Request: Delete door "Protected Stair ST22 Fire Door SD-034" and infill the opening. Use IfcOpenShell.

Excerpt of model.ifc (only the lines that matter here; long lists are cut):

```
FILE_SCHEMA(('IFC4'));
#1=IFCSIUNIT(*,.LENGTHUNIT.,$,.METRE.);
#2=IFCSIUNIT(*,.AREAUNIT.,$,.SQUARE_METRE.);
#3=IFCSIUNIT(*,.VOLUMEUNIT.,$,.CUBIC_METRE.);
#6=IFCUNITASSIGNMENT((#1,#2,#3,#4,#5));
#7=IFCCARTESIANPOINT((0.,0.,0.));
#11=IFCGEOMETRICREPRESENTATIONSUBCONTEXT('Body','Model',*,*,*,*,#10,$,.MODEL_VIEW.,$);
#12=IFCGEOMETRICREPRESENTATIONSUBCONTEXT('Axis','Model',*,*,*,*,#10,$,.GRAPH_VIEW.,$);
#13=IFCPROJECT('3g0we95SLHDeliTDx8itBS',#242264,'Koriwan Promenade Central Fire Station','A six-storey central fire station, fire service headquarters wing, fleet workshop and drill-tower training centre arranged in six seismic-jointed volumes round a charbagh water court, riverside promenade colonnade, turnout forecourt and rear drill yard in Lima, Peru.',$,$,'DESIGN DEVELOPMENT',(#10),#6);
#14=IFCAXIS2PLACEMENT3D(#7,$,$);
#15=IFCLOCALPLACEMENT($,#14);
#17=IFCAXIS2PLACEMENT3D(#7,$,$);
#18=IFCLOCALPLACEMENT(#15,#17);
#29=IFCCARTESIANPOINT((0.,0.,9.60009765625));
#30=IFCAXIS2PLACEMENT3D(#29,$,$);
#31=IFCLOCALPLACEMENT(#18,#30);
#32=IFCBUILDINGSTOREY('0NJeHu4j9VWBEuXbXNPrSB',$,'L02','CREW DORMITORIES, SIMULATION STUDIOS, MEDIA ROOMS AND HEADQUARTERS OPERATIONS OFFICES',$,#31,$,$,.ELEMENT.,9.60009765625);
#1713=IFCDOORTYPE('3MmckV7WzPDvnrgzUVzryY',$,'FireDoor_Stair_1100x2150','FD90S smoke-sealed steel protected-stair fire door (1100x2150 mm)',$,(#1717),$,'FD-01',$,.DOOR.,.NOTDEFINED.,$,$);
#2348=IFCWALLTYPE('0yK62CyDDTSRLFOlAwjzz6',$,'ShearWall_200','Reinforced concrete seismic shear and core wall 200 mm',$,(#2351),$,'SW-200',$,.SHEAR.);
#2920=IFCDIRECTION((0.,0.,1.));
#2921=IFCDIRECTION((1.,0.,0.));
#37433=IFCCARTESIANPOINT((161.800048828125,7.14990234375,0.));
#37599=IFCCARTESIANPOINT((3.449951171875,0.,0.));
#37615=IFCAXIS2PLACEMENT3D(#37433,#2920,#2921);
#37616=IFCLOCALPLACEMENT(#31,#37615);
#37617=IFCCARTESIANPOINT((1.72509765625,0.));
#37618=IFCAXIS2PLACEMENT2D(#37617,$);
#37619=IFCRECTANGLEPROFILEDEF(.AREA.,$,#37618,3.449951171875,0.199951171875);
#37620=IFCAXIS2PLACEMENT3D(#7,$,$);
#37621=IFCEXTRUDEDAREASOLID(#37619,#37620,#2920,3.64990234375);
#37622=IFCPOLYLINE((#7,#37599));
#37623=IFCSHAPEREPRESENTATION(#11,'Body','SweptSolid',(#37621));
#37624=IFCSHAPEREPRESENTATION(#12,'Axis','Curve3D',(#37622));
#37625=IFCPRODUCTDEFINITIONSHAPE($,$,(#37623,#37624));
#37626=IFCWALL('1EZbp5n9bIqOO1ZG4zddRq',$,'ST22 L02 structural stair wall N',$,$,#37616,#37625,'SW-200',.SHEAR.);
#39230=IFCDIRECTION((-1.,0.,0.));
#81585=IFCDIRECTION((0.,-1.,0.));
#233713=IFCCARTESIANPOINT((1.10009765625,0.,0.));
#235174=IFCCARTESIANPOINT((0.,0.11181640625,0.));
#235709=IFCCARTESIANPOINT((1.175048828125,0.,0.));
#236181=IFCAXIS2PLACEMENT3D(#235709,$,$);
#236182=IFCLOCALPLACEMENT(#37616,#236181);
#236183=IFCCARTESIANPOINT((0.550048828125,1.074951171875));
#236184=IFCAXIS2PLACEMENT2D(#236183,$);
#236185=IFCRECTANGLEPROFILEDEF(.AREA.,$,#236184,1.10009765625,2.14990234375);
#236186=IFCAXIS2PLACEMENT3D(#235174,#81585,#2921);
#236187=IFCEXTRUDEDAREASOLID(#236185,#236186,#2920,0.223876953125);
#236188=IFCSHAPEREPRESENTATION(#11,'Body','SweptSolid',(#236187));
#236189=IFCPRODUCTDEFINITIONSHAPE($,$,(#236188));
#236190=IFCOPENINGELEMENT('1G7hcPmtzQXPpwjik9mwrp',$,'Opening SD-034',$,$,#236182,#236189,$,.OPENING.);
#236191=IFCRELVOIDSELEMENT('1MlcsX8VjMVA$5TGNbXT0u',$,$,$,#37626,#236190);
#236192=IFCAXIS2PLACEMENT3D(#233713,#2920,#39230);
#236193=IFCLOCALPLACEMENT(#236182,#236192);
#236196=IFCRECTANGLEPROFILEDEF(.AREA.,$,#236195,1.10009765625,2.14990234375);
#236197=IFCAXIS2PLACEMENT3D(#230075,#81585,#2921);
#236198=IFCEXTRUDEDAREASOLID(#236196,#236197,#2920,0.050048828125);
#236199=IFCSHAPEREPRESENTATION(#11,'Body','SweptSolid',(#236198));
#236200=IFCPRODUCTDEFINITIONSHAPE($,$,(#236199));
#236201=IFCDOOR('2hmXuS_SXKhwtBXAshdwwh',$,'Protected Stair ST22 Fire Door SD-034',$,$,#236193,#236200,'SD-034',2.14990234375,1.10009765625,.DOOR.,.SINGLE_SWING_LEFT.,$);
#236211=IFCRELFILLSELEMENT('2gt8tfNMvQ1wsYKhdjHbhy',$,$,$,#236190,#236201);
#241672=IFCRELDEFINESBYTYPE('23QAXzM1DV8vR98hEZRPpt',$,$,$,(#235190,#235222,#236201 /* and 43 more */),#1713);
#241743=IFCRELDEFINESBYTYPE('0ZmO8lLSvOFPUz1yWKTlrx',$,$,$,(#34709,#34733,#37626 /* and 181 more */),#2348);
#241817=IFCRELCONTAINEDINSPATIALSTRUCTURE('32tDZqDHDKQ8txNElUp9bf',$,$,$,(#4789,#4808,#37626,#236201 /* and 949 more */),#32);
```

```python
import ifcopenshell
import ifcopenshell.api.feature
import ifcopenshell.api.root
import ifcopenshell.geom
import ifcopenshell.util.shape

model = ifcopenshell.open("model.ifc")
settings = ifcopenshell.geom.settings()


def volume(element):
    """Net volume in cubic metres, openings subtracted."""
    shape = ifcopenshell.geom.create_shape(settings, element)
    return ifcopenshell.util.shape.get_volume(shape.geometry)


door = model.by_guid("2hmXuS_SXKhwtBXAshdwwh")
opening = door.FillsVoids[0].RelatingOpeningElement
wall = opening.VoidsElements[0].RelatingBuildingElement
before = volume(wall)

ifcopenshell.api.root.remove_product(model, product=door)
ifcopenshell.api.feature.remove_feature(model, feature=opening)

after = volume(wall)

print(f"wall volume {before:.3f} -> {after:.3f} m3")

model.write("model_updated.ifc")
```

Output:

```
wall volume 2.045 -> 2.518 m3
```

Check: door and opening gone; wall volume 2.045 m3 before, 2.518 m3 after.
